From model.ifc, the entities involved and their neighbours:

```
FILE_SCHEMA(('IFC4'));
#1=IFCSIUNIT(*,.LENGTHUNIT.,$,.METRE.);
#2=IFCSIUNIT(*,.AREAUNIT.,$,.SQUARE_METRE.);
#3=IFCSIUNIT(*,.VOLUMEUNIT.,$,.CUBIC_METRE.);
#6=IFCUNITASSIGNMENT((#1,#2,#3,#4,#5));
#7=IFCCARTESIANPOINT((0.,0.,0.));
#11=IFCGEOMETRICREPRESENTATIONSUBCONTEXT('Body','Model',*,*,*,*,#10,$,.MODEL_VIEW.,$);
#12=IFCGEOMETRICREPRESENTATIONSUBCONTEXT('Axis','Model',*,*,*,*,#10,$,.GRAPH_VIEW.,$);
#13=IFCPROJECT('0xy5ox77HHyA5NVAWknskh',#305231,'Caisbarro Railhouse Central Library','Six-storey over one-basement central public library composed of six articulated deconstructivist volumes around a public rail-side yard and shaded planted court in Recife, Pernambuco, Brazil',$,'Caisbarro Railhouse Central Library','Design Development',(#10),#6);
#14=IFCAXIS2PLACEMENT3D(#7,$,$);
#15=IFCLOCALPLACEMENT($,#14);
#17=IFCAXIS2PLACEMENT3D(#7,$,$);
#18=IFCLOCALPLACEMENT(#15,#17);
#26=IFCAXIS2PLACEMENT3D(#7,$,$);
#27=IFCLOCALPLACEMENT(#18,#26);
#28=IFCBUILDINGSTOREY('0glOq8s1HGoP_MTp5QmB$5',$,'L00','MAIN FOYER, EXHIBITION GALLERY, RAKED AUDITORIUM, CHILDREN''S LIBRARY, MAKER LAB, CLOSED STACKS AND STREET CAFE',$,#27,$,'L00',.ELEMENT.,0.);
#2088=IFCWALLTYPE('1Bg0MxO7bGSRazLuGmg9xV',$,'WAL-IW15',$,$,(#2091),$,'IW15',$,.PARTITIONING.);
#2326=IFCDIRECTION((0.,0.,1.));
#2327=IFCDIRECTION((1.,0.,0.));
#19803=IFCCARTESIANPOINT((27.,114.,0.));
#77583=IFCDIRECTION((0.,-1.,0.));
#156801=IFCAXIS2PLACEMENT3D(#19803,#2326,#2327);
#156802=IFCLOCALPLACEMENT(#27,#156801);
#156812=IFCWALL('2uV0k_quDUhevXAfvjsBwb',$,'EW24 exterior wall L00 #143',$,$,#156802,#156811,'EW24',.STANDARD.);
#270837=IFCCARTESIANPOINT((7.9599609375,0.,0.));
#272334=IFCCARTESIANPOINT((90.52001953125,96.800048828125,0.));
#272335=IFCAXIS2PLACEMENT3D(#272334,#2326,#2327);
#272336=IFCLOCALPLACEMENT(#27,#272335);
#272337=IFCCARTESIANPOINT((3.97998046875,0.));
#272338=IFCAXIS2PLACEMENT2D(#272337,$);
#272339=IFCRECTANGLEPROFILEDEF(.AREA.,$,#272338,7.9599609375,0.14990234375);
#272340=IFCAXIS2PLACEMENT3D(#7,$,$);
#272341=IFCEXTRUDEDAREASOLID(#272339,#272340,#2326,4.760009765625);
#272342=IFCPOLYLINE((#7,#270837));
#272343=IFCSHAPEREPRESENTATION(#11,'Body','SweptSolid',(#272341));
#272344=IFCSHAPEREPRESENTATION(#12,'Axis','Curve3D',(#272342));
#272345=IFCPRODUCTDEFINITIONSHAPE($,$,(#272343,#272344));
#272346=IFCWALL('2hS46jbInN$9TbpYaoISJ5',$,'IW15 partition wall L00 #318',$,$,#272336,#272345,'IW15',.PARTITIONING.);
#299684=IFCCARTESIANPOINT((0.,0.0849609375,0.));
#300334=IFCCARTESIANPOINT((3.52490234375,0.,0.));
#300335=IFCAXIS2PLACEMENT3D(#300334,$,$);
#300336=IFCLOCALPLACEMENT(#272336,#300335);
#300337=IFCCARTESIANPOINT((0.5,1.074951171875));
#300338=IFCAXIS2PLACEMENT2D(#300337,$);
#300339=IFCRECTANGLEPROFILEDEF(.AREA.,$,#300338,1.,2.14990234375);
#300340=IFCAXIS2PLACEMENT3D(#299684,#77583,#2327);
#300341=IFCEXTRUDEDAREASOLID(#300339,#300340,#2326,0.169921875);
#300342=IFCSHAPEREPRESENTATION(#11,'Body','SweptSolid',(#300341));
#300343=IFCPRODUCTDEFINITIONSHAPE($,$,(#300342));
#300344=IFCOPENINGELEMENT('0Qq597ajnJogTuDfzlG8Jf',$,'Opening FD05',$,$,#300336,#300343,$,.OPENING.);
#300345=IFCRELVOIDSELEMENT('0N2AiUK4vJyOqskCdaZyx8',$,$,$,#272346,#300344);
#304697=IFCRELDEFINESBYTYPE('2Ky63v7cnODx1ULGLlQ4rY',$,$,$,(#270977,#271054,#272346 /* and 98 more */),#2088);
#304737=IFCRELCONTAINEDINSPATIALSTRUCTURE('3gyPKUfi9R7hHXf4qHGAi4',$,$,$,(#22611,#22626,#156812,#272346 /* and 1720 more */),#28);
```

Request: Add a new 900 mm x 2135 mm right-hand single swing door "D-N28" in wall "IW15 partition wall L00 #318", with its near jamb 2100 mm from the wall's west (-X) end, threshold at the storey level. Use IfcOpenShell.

```python
import numpy as np
import ifcopenshell
import ifcopenshell.api.feature
import ifcopenshell.api.geometry
import ifcopenshell.api.root
import ifcopenshell.api.spatial
import ifcopenshell.geom
import ifcopenshell.util.element
import ifcopenshell.util.placement
import ifcopenshell.util.representation
import ifcopenshell.util.shape
import ifcopenshell.util.unit

model = ifcopenshell.open("model.ifc")
unit_scale = ifcopenshell.util.unit.calculate_unit_scale(model)
settings = ifcopenshell.geom.settings()


def volume(element):
    """Net volume in cubic metres, openings subtracted."""
    shape = ifcopenshell.geom.create_shape(settings, element)
    return ifcopenshell.util.shape.get_volume(shape.geometry)


wall = model.by_guid("2hS46jbInN$9TbpYaoISJ5")
storey = ifcopenshell.util.element.get_container(wall, ifc_class="IfcBuildingStorey")
context = ifcopenshell.util.representation.get_context(model, "Model", "Body", "MODEL_VIEW")
before = volume(wall)

width, height, from_end, sill = 0.9, 2.135, 2.1, 0.0  # metres

# The wall runs along its own X axis, and the end named is its -X end.
wall_shape = ifcopenshell.geom.create_shape(settings, wall)
x, y, z = ifcopenshell.util.shape.get_vertices(wall_shape.geometry).T
start = x.min() + from_end
face, thickness = float(y.min()), float(y.max() - y.min())
wall_matrix = ifcopenshell.util.placement.get_local_placement(wall.ObjectPlacement)
level = ifcopenshell.util.placement.get_local_placement(storey.ObjectPlacement)[2, 3]


def in_wall(x, y):
    """Placement at x, y metres in the wall's axes, at sill height."""
    matrix = wall_matrix.copy()
    matrix[:, 3] = wall_matrix @ np.array([x / unit_scale, y / unit_scale, 0.0, 1.0])
    matrix[2, 3] = level + sill / unit_scale
    return matrix


# Opening: a box that overshoots both wall faces by 50 mm.
opening = ifcopenshell.api.root.create_entity(model, ifc_class="IfcOpeningElement", predefined_type="OPENING")
box = ifcopenshell.api.geometry.add_wall_representation(
    model, context=context, length=width, height=height, thickness=thickness + 0.1
)
ifcopenshell.api.geometry.assign_representation(model, product=opening, representation=box)
ifcopenshell.api.geometry.edit_object_placement(model, product=opening, matrix=in_wall(start, face - 0.05), is_si=False)
ifcopenshell.api.feature.add_feature(model, feature=opening, element=wall)

door = ifcopenshell.api.root.create_entity(model, ifc_class="IfcDoor", name="D-N28", predefined_type="DOOR")
door.OverallWidth, door.OverallHeight = width / unit_scale, height / unit_scale
door.OperationType = "SINGLE_SWING_RIGHT"
body = ifcopenshell.api.geometry.add_door_representation(
    model,
    context=context,
    overall_width=door.OverallWidth,
    overall_height=door.OverallHeight,
    operation_type="SINGLE_SWING_RIGHT",
    lining_properties={"LiningDepth": thickness / unit_scale, "ThresholdDepth": thickness / unit_scale},
)
ifcopenshell.api.geometry.assign_representation(model, product=door, representation=body)
ifcopenshell.api.spatial.assign_container(model, products=[door], relating_structure=storey)
ifcopenshell.api.feature.add_filling(model, opening=opening, element=door)

# The lining spans the wall, so the door starts at the wall face.
ifcopenshell.api.geometry.edit_object_placement(model, product=door, matrix=in_wall(start, face), is_si=False)

after = volume(wall)

print(f"wall volume {before:.3f} -> {after:.3f} m3")

model.write("model_v2.ifc")
```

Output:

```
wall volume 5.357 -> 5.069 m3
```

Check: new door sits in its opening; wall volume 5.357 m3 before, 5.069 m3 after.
